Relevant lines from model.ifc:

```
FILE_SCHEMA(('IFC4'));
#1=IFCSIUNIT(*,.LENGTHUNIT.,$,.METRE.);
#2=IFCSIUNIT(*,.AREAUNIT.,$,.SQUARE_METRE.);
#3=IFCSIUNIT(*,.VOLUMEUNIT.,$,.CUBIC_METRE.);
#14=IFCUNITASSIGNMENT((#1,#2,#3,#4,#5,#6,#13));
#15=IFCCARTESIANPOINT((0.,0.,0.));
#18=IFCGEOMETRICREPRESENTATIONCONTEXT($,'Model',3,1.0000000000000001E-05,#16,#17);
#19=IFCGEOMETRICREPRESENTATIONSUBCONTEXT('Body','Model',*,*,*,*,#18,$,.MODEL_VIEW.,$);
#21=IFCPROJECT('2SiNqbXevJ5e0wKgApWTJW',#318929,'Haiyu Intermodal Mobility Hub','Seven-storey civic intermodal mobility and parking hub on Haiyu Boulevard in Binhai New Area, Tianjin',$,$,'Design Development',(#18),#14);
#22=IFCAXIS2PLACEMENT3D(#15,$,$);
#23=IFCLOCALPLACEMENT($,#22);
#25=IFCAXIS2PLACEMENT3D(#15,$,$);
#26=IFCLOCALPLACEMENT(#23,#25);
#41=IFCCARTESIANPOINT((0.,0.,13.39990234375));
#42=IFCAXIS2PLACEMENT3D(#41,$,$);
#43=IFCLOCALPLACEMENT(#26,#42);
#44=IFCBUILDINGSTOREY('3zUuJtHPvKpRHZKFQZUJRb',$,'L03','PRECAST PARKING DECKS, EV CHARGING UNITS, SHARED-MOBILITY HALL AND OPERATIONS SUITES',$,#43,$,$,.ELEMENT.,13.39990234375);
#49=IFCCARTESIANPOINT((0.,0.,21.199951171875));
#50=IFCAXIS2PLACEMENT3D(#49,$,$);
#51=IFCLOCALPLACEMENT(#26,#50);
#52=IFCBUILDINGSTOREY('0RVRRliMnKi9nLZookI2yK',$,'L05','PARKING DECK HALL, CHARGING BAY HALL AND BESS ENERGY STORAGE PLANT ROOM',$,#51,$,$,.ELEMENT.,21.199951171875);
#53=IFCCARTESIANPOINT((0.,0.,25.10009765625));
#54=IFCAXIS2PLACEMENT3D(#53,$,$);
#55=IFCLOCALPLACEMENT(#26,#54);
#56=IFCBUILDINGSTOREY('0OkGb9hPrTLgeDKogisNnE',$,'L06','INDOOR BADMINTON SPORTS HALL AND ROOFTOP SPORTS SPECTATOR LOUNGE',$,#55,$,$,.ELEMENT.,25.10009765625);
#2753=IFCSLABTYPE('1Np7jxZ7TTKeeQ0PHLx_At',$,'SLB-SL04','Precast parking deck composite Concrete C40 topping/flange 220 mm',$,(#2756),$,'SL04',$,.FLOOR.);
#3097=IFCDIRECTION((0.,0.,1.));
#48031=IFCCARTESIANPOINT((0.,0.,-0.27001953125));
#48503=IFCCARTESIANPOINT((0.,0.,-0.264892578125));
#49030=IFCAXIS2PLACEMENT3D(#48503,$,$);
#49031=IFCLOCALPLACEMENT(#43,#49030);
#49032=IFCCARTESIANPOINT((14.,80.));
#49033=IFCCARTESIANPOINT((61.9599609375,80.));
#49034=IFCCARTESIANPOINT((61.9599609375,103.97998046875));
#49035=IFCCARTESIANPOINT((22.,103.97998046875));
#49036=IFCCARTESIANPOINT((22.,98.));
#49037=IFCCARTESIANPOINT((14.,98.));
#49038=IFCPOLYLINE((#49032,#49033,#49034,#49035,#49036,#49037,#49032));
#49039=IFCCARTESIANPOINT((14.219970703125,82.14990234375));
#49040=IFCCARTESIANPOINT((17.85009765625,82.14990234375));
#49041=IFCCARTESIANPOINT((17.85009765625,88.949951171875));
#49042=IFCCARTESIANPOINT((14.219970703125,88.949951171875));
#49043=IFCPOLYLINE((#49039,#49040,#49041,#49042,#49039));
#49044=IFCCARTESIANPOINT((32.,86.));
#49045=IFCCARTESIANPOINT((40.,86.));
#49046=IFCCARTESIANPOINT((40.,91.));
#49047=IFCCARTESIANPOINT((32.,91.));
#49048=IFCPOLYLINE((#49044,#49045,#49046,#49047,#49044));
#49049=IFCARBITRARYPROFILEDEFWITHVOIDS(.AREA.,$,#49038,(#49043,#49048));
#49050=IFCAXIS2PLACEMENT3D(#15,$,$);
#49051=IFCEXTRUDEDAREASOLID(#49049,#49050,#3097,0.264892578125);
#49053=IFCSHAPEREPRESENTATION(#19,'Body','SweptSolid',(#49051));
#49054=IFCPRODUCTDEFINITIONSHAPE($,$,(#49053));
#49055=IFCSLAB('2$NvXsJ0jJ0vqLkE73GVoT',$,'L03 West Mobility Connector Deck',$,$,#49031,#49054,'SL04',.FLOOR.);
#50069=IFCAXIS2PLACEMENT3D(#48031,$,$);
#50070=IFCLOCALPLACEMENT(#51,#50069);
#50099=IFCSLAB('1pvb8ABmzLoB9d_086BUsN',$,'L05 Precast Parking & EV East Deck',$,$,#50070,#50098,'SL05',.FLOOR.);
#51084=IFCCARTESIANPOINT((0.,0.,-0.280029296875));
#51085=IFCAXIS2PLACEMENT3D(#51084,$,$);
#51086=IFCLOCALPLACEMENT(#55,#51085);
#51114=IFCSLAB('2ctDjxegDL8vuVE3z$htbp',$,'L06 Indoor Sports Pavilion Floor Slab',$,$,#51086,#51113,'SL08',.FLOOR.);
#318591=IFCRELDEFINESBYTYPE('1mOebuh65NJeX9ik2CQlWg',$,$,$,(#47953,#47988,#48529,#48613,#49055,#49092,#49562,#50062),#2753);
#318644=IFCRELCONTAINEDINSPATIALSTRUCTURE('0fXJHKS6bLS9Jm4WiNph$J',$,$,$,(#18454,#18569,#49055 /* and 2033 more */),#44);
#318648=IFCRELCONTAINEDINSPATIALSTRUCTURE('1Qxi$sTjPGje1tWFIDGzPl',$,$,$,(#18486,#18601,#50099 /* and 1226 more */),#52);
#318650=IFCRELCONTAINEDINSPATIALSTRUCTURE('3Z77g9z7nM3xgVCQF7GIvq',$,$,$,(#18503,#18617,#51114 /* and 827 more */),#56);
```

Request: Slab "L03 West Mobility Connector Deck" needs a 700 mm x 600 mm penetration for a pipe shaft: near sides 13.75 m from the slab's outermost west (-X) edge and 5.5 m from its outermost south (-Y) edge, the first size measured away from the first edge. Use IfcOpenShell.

```python
import numpy as np
import ifcopenshell
import ifcopenshell.api.feature
import ifcopenshell.api.geometry
import ifcopenshell.api.root
import ifcopenshell.geom
import ifcopenshell.util.placement
import ifcopenshell.util.representation
import ifcopenshell.util.shape
import ifcopenshell.util.unit

model = ifcopenshell.open("model.ifc")
unit_scale = ifcopenshell.util.unit.calculate_unit_scale(model)
settings = ifcopenshell.geom.settings()


def volume(element):
    """Net volume in cubic metres, openings subtracted."""
    shape = ifcopenshell.geom.create_shape(settings, element)
    return ifcopenshell.util.shape.get_volume(shape.geometry)


slab = model.by_guid("2$NvXsJ0jJ0vqLkE73GVoT")
before = volume(slab)

# Extent in the slab's own axes, in metres. The edges named are its -X and -Y sides.
slab_shape = ifcopenshell.geom.create_shape(settings, slab)
vertices = ifcopenshell.util.shape.get_vertices(slab_shape.geometry)
x_min, y_min, bottom = vertices.min(axis=0)
top = vertices[:, 2].max()

opening = ifcopenshell.api.root.create_entity(model, ifc_class="IfcOpeningElement", name="Pipe shaft opening", predefined_type="OPENING")
context = ifcopenshell.util.representation.get_context(model, "Model", "Body", "MODEL_VIEW")
width, depth = 0.7, 0.6
outline = [(0.0, 0.0), (width, 0.0), (width, depth), (0.0, depth), (0.0, 0.0)]
# Overshoot both faces by 50 mm so the cut is clean.
shape = ifcopenshell.api.geometry.add_slab_representation(
    model, context=context, depth=top - bottom + 0.1, polyline=outline
)
ifcopenshell.api.geometry.assign_representation(model, product=opening, representation=shape)

matrix = ifcopenshell.util.placement.get_local_placement(slab.ObjectPlacement)
matrix[:, 3] = matrix @ np.append(np.array([x_min + 13.75, y_min + 5.5, bottom - 0.05]) / unit_scale, 1.0)
ifcopenshell.api.geometry.edit_object_placement(model, product=opening, matrix=matrix, is_si=False)
ifcopenshell.api.feature.add_feature(model, feature=opening, element=slab)

after = volume(slab)

print(f"slab volume {before:.3f} -> {after:.3f} m3")

model.write("model_rev.ifc")
```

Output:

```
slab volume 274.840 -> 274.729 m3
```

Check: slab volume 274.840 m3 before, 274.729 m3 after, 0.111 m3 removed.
